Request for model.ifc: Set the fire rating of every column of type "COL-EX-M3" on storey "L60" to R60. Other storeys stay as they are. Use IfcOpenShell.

First a look at what the model holds.

```python
import ifcopenshell
import ifcopenshell.util.element

model = ifcopenshell.open("model.ifc")
print(model.schema)
storey = next(s for s in model.by_type("IfcBuildingStorey") if s.Name == "L60")
columns = [e for e in ifcopenshell.util.element.get_decomposition(storey) if e.is_a("IfcColumn")]
seen = {}
for e in columns:
    element_type = ifcopenshell.util.element.get_type(e)
    key = (element_type.Name if element_type != e and element_type else None, ifcopenshell.util.element.get_pset(e, "Pset_ColumnCommon", "FireRating"))
    seen[key] = seen.get(key, 0) + 1
for (name, value), count in sorted(seen.items(), key=str):
    print(count, "x", name, "|", value)
```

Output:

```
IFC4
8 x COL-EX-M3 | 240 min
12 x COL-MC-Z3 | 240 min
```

```python
import ifcopenshell
import ifcopenshell.api.pset
import ifcopenshell.util.element

model = ifcopenshell.open("model.ifc")

storey = next(s for s in model.by_type("IfcBuildingStorey") if s.Name == "L60")
columns = [e for e in ifcopenshell.util.element.get_decomposition(storey) if e.is_a("IfcColumn")]

count = 0
for e in columns:
    element_type = ifcopenshell.util.element.get_type(e)
    if element_type in (None, e) or element_type.Name != "COL-EX-M3":
        continue
    found = ifcopenshell.util.element.get_pset(e, "Pset_ColumnCommon", should_inherit=False)
    if found:
        pset = model.by_id(found["id"])
        if len(ifcopenshell.util.element.get_elements_by_pset(pset)) > 1:
            pset = ifcopenshell.api.pset.unshare_pset(model, products=[e], pset=pset)[0]
    else:
        pset = ifcopenshell.api.pset.add_pset(model, product=e, name="Pset_ColumnCommon")
    ifcopenshell.api.pset.edit_pset(model, pset=pset, properties={"FireRating": "R60"})
    count += 1

print(count, "columns updated")

model.write("model_rev.ifc")
```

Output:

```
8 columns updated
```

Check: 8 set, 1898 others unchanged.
